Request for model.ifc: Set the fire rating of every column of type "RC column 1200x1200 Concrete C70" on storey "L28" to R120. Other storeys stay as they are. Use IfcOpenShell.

First a look at what the model holds.

```python
import ifcopenshell
import ifcopenshell.util.element

model = ifcopenshell.open("model.ifc")
print(model.schema)
storey = next(s for s in model.by_type("IfcBuildingStorey") if s.Name == "L28")
columns = [e for e in ifcopenshell.util.element.get_decomposition(storey) if e.is_a("IfcColumn")]
seen = {}
for e in columns:
    element_type = ifcopenshell.util.element.get_type(e)
    key = (element_type.Name if element_type != e and element_type else None, ifcopenshell.util.element.get_pset(e, "Pset_ColumnCommon", "FireRating"))
    seen[key] = seen.get(key, 0) + 1
for (name, value), count in sorted(seen.items(), key=str):
    print(count, "x", name, "|", value)
```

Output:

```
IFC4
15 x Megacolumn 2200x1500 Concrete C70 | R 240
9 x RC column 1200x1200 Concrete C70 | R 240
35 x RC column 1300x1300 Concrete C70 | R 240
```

```python
import ifcopenshell
import ifcopenshell.api.pset
import ifcopenshell.util.element

model = ifcopenshell.open("model.ifc")

storey = next(s for s in model.by_type("IfcBuildingStorey") if s.Name == "L28")
columns = [e for e in ifcopenshell.util.element.get_decomposition(storey) if e.is_a("IfcColumn")]

count = 0
for e in columns:
    element_type = ifcopenshell.util.element.get_type(e)
    if element_type in (None, e) or element_type.Name != "RC column 1200x1200 Concrete C70":
        continue
    found = ifcopenshell.util.element.get_pset(e, "Pset_ColumnCommon", should_inherit=False)
    if found:
        pset = model.by_id(found["id"])
        if len(ifcopenshell.util.element.get_elements_by_pset(pset)) > 1:
            pset = ifcopenshell.api.pset.unshare_pset(model, products=[e], pset=pset)[0]
    else:
        pset = ifcopenshell.api.pset.add_pset(model, product=e, name="Pset_ColumnCommon")
    ifcopenshell.api.pset.edit_pset(model, pset=pset, properties={"FireRating": "R120"})
    count += 1

print(count, "columns updated")

model.write("model_edited.ifc")
```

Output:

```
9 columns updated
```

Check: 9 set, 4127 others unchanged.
